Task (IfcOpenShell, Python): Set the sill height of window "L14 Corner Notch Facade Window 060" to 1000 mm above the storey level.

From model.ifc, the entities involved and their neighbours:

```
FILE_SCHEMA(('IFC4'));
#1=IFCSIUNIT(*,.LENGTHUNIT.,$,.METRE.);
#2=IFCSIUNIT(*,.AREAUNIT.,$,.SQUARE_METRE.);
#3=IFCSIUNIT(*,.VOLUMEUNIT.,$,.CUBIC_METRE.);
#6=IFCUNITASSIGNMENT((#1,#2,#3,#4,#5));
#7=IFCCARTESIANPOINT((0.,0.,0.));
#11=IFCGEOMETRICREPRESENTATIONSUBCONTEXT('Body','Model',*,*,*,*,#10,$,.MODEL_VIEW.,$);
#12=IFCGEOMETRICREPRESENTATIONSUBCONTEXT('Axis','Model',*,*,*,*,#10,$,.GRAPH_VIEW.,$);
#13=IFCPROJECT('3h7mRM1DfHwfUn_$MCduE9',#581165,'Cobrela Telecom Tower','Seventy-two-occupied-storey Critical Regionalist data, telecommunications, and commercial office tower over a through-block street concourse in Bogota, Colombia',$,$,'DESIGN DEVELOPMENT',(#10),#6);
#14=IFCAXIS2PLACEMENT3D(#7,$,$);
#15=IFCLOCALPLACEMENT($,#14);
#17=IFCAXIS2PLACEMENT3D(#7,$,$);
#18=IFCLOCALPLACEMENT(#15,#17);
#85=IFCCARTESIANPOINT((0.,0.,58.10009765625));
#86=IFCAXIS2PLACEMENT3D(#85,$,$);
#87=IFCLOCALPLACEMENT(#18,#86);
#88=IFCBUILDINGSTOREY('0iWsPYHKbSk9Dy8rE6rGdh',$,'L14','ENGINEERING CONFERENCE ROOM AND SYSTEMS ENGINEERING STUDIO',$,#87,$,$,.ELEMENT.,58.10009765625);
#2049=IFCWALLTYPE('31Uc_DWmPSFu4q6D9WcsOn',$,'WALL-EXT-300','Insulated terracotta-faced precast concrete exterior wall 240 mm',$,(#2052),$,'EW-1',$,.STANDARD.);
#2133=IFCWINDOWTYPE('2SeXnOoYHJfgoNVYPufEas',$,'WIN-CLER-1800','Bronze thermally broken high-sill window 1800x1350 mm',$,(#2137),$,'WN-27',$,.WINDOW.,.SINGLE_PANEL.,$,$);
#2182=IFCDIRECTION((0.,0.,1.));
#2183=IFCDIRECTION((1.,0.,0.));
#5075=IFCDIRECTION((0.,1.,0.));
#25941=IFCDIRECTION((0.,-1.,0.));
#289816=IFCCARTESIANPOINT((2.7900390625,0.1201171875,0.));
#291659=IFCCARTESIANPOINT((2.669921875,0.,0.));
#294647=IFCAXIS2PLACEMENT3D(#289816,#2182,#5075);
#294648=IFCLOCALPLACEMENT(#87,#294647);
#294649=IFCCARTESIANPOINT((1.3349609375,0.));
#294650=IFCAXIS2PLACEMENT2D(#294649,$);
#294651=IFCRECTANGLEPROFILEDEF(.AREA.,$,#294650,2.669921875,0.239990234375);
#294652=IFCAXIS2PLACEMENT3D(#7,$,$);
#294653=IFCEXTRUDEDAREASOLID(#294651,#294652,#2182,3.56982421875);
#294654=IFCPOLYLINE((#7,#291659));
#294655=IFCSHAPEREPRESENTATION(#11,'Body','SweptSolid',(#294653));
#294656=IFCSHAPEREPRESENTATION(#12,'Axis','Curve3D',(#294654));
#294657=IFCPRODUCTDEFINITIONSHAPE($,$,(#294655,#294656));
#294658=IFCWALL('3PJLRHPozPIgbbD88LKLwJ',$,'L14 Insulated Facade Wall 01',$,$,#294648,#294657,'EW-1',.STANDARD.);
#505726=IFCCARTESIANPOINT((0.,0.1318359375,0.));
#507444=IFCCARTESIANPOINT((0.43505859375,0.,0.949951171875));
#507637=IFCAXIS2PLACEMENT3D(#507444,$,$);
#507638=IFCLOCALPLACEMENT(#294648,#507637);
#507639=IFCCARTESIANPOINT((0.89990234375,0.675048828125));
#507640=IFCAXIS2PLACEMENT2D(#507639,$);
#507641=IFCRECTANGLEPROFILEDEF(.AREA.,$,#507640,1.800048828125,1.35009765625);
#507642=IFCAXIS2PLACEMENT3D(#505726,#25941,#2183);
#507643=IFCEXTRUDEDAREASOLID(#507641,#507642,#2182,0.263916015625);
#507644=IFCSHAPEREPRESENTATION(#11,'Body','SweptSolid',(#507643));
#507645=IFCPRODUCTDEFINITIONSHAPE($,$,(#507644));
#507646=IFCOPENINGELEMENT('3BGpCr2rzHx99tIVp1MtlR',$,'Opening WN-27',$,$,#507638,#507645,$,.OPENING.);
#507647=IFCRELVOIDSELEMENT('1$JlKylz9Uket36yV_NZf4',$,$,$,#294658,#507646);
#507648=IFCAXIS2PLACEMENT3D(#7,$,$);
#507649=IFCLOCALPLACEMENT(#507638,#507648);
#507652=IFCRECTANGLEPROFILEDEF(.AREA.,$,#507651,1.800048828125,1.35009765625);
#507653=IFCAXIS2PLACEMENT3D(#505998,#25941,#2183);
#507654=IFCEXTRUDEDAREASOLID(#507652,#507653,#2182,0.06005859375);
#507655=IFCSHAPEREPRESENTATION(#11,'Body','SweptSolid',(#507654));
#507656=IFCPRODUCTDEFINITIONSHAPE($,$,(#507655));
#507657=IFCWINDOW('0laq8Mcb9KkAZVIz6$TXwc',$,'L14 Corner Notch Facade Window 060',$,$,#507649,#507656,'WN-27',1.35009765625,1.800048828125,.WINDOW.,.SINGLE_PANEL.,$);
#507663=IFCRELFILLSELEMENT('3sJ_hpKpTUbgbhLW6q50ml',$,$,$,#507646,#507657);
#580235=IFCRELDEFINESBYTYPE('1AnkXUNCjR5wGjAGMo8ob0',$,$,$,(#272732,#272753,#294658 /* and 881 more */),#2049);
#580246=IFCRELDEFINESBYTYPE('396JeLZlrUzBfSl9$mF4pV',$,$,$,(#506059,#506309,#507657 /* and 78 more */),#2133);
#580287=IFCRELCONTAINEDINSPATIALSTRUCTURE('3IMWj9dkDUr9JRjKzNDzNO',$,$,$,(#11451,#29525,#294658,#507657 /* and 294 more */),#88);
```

```python
import numpy as np
import ifcopenshell
import ifcopenshell.api.geometry
import ifcopenshell.geom
import ifcopenshell.util.element
import ifcopenshell.util.placement
import ifcopenshell.util.shape
import ifcopenshell.util.unit

model = ifcopenshell.open("model.ifc")
unit_scale = ifcopenshell.util.unit.calculate_unit_scale(model)

window = model.by_id(507657)
opening = window.FillsVoids[0].RelatingOpeningElement
storey = ifcopenshell.util.element.get_container(window, ifc_class="IfcBuildingStorey")
level = ifcopenshell.util.placement.get_local_placement(storey.ObjectPlacement)[2, 3]

# The opening's origin need not be at the sill, so measure its lowest point.
shape = ifcopenshell.geom.create_shape(ifcopenshell.geom.settings(), opening)
bottom = ifcopenshell.util.shape.get_shape_bottom_elevation(shape, shape.geometry) / unit_scale
dz = level + 1 / unit_scale - bottom

shift = np.array([0.0, 0.0, dz])
# The window is placed relative to its opening, so it follows when the opening moves.
matrix = ifcopenshell.util.placement.get_local_placement(opening.ObjectPlacement)
matrix[:3, 3] += shift
ifcopenshell.api.geometry.edit_object_placement(
    model, product=opening, matrix=matrix, is_si=False, should_transform_children=True
)

print(f"moved by {dz * unit_scale:+.3f} m")

model.write("model_edited.ifc")
```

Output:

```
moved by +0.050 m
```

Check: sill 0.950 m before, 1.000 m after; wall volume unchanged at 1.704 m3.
